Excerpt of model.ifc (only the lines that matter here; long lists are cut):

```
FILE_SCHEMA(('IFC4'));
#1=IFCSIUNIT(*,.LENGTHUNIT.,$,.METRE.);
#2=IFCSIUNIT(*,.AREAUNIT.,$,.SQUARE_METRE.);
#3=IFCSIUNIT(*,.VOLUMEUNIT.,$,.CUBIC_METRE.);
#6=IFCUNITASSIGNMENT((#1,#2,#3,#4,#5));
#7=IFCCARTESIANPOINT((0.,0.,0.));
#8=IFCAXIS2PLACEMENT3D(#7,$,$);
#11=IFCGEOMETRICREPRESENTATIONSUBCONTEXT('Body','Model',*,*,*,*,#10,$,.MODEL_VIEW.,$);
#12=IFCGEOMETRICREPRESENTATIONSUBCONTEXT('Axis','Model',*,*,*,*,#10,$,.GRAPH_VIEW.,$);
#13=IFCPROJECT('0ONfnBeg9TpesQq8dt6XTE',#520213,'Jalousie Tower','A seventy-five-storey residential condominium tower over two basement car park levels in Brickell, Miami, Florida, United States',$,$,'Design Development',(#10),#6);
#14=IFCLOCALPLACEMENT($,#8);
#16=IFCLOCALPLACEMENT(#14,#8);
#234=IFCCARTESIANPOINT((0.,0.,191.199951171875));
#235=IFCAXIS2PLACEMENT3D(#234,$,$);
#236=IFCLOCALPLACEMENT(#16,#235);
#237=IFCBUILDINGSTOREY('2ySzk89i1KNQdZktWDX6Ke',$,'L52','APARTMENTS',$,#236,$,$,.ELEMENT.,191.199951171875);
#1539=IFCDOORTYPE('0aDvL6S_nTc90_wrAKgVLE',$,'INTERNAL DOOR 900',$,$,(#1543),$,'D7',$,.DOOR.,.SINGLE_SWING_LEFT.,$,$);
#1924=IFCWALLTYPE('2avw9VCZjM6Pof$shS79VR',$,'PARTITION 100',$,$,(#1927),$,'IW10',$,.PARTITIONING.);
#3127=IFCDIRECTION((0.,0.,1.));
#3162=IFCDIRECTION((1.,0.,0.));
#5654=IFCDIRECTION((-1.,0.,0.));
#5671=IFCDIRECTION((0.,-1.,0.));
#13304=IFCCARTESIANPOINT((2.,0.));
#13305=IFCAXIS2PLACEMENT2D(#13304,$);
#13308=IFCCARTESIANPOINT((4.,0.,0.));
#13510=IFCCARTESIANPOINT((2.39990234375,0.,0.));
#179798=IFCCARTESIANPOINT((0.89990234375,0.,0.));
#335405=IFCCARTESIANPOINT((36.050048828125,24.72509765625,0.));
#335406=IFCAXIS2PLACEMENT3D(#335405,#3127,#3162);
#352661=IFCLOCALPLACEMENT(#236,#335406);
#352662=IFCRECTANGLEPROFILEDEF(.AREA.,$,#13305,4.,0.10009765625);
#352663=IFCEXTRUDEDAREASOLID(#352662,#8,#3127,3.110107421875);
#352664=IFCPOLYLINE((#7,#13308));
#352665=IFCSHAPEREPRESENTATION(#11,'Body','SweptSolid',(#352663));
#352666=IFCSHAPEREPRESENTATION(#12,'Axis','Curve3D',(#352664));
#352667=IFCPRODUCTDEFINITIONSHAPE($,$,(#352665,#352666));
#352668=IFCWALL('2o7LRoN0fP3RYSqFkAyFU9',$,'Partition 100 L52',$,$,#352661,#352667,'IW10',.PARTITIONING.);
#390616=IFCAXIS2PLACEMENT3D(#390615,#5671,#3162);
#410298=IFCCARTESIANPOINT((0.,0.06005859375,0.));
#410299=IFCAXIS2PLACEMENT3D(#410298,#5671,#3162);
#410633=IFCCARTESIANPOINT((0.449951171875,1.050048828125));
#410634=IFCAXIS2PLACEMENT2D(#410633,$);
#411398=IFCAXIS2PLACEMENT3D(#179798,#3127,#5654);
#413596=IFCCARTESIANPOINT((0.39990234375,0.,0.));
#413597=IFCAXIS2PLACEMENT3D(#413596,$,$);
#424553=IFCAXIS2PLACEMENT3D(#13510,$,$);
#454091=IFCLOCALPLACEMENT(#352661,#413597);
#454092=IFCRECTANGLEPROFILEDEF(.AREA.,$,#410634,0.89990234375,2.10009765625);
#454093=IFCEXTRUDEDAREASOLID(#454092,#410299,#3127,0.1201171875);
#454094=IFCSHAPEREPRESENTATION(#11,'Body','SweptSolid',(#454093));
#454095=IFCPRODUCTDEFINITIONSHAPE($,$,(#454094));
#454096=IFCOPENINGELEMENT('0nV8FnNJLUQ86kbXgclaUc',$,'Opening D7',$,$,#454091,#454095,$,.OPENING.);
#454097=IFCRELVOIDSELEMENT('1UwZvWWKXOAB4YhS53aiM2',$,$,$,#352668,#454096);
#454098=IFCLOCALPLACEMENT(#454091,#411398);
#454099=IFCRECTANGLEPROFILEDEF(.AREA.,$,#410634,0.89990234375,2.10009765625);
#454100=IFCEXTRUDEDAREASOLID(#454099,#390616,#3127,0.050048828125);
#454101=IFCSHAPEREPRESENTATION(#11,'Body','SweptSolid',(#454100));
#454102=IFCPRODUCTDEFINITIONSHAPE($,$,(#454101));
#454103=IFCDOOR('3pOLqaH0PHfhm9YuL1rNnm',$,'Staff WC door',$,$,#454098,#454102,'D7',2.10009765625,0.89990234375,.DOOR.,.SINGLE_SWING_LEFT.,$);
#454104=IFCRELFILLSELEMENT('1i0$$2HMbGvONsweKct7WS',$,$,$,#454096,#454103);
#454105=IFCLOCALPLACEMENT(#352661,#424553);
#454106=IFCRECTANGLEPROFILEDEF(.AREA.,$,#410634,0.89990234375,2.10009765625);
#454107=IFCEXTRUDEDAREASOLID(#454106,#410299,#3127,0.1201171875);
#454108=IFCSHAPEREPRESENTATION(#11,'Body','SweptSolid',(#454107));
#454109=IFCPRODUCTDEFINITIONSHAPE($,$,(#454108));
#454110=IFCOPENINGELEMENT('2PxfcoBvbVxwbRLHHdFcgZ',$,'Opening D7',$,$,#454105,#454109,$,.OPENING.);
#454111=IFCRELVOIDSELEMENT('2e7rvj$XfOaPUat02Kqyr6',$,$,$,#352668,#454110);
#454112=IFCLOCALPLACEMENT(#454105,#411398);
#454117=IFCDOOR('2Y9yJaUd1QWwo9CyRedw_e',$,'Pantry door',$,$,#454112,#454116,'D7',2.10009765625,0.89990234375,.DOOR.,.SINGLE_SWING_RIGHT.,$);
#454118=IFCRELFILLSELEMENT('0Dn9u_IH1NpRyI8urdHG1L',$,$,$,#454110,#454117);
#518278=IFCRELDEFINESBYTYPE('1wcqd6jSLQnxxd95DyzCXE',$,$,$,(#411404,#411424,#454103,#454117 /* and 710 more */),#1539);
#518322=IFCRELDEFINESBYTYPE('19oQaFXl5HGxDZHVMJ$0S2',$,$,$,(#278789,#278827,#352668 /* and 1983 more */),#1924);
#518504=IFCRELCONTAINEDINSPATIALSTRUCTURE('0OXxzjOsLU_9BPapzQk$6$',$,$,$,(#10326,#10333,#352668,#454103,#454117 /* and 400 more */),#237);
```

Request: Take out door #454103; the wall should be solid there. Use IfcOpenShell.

```python
import ifcopenshell
import ifcopenshell.api.feature
import ifcopenshell.api.root
import ifcopenshell.geom
import ifcopenshell.util.shape

model = ifcopenshell.open("model.ifc")
settings = ifcopenshell.geom.settings()


def volume(element):
    """Net volume in cubic metres, openings subtracted."""
    shape = ifcopenshell.geom.create_shape(settings, element)
    return ifcopenshell.util.shape.get_volume(shape.geometry)


door = model.by_id(454103)
opening = door.FillsVoids[0].RelatingOpeningElement
wall = opening.VoidsElements[0].RelatingBuildingElement
before = volume(wall)

ifcopenshell.api.root.remove_product(model, product=door)
ifcopenshell.api.feature.remove_feature(model, feature=opening)

after = volume(wall)

print(f"wall volume {before:.3f} -> {after:.3f} m3")

model.write("model_rev.ifc")
```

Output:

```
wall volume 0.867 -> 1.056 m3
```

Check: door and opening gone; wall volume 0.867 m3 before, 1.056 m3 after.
